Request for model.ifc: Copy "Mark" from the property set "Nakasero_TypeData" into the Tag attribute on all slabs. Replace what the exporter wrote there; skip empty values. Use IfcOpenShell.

First a look at what the model holds.

```python
import ifcopenshell
import ifcopenshell.util.element

model = ifcopenshell.open("model.ifc")
print(model.schema)
slabs = model.by_type("IfcSlab")
print(len(slabs), "slabs")
for e in slabs[:8]:
    source = ifcopenshell.util.element.get_pset(e, "Nakasero_TypeData", "Mark")
    target = e.Tag
    print(e.id(), repr(source), repr(target), sep=" | ")
```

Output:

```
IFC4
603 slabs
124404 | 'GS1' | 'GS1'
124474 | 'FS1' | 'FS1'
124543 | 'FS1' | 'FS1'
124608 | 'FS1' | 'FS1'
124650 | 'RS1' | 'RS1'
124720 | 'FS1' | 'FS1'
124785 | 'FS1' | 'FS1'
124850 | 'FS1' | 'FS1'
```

```python
import ifcopenshell
import ifcopenshell.util.element

model = ifcopenshell.open("model.ifc")

count = 0
for e in model.by_type("IfcSlab"):
    value = ifcopenshell.util.element.get_pset(e, "Nakasero_TypeData", "Mark")
    current = e.Tag
    if not value or not value.strip() or current == value:
        continue
    e.Tag = value
    count += 1

print(count, "slabs updated")

model.write("model_v2.ifc")
```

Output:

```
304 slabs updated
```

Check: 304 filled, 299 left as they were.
